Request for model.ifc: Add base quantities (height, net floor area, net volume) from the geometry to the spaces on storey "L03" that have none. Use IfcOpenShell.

First a look at what the model holds.

```python
import ifcopenshell
import ifcopenshell.util.element
import ifcopenshell.util.unit

model = ifcopenshell.open("model.ifc")
print(model.schema)
for unit_type in ("LENGTHUNIT", "AREAUNIT", "VOLUMEUNIT"):
    print(unit_type, ifcopenshell.util.unit.calculate_unit_scale(model, unit_type))
storey = next(s for s in model.by_type("IfcBuildingStorey") if s.Name == "L03")
spaces = [e for e in ifcopenshell.util.element.get_decomposition(storey) if e.is_a("IfcSpace")]
for e in sorted(spaces, key=lambda e: e.id()):
    print(e.id(), e.is_a(), e.Name, list(ifcopenshell.util.element.get_psets(e, qtos_only=True)), sep=" | ")
```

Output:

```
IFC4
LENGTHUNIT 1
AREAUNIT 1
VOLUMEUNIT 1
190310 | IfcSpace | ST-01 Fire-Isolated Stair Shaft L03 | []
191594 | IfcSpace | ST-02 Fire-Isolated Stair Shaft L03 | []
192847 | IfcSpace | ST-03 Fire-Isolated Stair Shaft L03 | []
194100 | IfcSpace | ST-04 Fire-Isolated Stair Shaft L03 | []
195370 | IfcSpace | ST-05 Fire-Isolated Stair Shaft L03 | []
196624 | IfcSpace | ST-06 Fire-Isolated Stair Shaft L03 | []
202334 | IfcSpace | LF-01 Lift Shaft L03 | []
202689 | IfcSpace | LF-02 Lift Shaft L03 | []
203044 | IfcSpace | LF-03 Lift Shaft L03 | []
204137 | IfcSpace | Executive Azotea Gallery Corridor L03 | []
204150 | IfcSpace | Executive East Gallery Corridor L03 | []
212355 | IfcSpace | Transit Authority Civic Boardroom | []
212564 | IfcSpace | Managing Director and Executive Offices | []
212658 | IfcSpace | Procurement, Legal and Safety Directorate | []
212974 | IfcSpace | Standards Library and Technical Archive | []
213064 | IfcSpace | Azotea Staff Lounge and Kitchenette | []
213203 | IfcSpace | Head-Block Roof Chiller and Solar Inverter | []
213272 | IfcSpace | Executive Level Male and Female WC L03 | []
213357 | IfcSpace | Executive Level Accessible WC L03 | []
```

```python
import ifcopenshell
import ifcopenshell.api.pset
import ifcopenshell.geom
import ifcopenshell.util.element
import ifcopenshell.util.shape
import ifcopenshell.util.unit

model = ifcopenshell.open("model.ifc")
unit_scale = ifcopenshell.util.unit.calculate_unit_scale(model)
area_scale = ifcopenshell.util.unit.calculate_unit_scale(model, "AREAUNIT")
volume_scale = ifcopenshell.util.unit.calculate_unit_scale(model, "VOLUMEUNIT")
settings = ifcopenshell.geom.settings()

storey = next(s for s in model.by_type("IfcBuildingStorey") if s.Name == "L03")
spaces = [e for e in ifcopenshell.util.element.get_decomposition(storey) if e.is_a("IfcSpace")]

for e in sorted(spaces, key=lambda e: e.id()):
    if ifcopenshell.util.element.get_psets(e, qtos_only=True, should_inherit=False):
        continue
    # Geometry comes back in metres, in the element's own axes.
    shape = ifcopenshell.geom.create_shape(settings, e)
    values = {
        "Height": ifcopenshell.util.shape.get_z(shape.geometry) / unit_scale,
        "NetFloorArea": ifcopenshell.util.shape.get_footprint_area(shape.geometry) / area_scale,
        "NetVolume": ifcopenshell.util.shape.get_volume(shape.geometry) / volume_scale,
    }
    qto = ifcopenshell.api.pset.add_qto(model, product=e, name="Qto_SpaceBaseQuantities")
    ifcopenshell.api.pset.edit_qto(model, qto=qto, properties=values)
    print(e.id(), {k: round(v, 3) for k, v in values.items()})

model.write("model_updated.ifc")
```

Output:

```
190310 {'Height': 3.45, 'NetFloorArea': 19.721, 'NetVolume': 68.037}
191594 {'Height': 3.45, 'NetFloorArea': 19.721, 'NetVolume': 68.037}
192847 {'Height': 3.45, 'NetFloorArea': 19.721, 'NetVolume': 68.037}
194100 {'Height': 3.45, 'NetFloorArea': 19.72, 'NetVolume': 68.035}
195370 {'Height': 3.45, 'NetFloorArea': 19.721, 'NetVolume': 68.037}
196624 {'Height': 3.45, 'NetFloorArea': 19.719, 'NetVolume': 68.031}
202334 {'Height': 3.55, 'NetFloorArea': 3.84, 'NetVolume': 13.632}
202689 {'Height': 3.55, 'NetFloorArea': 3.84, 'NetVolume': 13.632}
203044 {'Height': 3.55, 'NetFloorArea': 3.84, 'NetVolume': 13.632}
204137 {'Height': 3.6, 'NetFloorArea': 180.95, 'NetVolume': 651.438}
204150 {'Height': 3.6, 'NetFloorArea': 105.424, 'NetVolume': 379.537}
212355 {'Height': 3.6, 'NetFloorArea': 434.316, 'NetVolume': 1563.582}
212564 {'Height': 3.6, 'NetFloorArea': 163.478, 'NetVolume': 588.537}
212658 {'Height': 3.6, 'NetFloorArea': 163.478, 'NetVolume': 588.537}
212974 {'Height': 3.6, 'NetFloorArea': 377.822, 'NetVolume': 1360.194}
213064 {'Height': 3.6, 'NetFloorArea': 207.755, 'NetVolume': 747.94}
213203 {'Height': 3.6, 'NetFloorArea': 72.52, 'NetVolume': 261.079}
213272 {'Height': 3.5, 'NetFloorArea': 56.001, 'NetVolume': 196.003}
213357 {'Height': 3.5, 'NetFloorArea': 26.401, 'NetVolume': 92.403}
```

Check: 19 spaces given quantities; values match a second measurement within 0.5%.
